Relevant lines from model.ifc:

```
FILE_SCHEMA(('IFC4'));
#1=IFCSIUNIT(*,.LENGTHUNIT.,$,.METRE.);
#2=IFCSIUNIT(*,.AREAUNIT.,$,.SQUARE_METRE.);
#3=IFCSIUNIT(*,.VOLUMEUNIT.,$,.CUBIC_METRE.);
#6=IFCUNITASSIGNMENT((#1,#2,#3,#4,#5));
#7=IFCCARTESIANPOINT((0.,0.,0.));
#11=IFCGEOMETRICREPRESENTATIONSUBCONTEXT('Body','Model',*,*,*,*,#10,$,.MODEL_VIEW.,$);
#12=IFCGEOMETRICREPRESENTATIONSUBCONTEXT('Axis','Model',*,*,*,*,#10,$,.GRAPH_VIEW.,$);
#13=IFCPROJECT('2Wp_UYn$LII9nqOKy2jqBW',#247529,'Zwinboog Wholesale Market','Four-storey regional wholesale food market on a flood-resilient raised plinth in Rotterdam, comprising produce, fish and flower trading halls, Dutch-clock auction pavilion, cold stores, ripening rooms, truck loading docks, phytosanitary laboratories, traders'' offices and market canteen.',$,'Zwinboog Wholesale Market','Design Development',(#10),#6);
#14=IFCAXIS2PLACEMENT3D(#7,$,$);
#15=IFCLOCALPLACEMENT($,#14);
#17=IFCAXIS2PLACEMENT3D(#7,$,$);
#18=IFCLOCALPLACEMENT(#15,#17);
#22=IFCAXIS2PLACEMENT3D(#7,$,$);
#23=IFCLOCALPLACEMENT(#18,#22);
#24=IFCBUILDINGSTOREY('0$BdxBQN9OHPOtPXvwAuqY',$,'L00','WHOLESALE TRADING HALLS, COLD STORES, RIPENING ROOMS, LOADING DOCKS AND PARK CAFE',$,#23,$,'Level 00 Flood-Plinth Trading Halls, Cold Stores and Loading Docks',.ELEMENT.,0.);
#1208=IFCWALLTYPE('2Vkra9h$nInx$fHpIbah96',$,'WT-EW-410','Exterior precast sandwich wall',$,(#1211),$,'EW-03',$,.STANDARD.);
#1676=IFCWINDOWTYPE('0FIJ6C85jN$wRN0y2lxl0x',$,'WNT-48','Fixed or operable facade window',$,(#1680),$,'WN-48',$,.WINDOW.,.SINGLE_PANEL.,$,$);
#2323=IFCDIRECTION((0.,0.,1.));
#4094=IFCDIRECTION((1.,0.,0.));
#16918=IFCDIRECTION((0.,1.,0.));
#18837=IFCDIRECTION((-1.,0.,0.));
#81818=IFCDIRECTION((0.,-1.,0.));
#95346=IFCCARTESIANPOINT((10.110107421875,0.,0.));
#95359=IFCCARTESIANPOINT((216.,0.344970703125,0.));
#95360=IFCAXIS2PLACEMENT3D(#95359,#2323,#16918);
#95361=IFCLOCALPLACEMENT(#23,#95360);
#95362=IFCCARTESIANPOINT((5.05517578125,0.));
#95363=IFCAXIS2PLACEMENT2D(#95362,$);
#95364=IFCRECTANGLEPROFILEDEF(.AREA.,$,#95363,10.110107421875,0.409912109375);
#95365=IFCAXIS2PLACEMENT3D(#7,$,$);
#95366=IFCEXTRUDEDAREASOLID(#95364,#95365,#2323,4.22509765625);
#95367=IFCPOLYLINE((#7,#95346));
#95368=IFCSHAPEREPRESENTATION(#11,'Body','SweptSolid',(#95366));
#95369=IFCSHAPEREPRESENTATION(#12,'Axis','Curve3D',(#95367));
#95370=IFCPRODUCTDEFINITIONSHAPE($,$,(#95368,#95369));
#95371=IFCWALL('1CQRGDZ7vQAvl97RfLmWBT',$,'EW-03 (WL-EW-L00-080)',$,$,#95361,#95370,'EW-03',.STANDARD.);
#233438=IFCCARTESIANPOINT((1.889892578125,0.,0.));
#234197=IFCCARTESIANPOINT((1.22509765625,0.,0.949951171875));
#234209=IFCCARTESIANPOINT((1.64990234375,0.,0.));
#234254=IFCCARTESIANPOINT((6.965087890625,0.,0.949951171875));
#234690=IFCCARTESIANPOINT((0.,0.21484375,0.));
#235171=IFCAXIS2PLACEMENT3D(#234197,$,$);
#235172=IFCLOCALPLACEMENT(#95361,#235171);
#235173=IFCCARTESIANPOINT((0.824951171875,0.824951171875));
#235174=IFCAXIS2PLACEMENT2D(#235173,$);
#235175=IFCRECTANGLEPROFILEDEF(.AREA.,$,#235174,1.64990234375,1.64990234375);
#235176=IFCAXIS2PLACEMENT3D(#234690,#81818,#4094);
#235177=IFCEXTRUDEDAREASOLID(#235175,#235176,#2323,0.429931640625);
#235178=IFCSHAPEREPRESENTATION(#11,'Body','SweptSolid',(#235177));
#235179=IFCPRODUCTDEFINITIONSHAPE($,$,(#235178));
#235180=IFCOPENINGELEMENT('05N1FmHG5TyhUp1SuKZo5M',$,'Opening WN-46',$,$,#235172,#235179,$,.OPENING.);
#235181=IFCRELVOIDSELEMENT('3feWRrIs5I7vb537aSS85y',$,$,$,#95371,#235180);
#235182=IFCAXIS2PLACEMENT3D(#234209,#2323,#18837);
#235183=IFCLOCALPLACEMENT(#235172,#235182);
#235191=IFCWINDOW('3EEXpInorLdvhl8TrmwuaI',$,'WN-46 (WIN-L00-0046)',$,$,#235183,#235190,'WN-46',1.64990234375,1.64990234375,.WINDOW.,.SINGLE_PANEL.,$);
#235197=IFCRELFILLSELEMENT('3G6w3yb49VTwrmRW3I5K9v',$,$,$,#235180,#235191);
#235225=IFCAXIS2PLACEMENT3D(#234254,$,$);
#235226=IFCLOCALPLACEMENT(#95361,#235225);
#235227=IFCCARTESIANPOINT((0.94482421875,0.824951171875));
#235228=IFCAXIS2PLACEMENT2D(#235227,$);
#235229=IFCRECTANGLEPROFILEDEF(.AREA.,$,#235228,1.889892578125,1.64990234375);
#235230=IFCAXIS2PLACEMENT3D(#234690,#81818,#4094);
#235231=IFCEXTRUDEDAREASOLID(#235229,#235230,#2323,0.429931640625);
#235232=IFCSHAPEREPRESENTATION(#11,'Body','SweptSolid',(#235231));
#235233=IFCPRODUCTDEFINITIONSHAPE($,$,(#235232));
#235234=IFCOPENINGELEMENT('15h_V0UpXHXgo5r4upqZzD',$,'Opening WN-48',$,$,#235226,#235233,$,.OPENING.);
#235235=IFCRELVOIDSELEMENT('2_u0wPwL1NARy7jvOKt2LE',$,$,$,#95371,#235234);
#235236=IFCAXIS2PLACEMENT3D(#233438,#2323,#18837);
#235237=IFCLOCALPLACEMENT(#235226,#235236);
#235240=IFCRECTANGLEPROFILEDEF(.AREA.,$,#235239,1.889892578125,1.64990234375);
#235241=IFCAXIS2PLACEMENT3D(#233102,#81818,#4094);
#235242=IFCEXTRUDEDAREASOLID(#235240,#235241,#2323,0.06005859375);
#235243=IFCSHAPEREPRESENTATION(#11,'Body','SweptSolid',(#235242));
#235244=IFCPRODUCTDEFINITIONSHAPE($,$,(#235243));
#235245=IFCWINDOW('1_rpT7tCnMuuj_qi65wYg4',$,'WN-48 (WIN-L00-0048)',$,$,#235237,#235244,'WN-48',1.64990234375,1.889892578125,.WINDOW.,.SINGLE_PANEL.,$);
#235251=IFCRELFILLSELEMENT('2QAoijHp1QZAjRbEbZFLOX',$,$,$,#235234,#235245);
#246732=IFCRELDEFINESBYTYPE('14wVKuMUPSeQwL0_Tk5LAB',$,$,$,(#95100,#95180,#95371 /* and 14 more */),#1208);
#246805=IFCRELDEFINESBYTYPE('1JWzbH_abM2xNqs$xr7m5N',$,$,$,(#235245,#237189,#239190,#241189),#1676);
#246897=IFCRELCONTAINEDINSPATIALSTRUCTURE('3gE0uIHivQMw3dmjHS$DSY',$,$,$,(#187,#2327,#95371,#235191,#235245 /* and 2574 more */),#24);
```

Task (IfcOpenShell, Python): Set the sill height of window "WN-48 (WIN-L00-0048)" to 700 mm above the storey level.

```python
import numpy as np
import ifcopenshell
import ifcopenshell.api.geometry
import ifcopenshell.geom
import ifcopenshell.util.element
import ifcopenshell.util.placement
import ifcopenshell.util.shape
import ifcopenshell.util.unit

model = ifcopenshell.open("model.ifc")
unit_scale = ifcopenshell.util.unit.calculate_unit_scale(model)

window = model.by_id(235245)
opening = window.FillsVoids[0].RelatingOpeningElement
storey = ifcopenshell.util.element.get_container(window, ifc_class="IfcBuildingStorey")
level = ifcopenshell.util.placement.get_local_placement(storey.ObjectPlacement)[2, 3]

# The opening's origin need not be at the sill, so measure its lowest point.
shape = ifcopenshell.geom.create_shape(ifcopenshell.geom.settings(), opening)
bottom = ifcopenshell.util.shape.get_shape_bottom_elevation(shape, shape.geometry) / unit_scale
dz = level + 0.7 / unit_scale - bottom

shift = np.array([0.0, 0.0, dz])
# The window is placed relative to its opening, so it follows when the opening moves.
matrix = ifcopenshell.util.placement.get_local_placement(opening.ObjectPlacement)
matrix[:3, 3] += shift
ifcopenshell.api.geometry.edit_object_placement(
    model, product=opening, matrix=matrix, is_si=False, should_transform_children=True
)

print(f"moved by {dz * unit_scale:+.3f} m")

model.write("model-out.ifc")
```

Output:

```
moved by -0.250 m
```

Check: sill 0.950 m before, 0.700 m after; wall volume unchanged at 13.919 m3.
